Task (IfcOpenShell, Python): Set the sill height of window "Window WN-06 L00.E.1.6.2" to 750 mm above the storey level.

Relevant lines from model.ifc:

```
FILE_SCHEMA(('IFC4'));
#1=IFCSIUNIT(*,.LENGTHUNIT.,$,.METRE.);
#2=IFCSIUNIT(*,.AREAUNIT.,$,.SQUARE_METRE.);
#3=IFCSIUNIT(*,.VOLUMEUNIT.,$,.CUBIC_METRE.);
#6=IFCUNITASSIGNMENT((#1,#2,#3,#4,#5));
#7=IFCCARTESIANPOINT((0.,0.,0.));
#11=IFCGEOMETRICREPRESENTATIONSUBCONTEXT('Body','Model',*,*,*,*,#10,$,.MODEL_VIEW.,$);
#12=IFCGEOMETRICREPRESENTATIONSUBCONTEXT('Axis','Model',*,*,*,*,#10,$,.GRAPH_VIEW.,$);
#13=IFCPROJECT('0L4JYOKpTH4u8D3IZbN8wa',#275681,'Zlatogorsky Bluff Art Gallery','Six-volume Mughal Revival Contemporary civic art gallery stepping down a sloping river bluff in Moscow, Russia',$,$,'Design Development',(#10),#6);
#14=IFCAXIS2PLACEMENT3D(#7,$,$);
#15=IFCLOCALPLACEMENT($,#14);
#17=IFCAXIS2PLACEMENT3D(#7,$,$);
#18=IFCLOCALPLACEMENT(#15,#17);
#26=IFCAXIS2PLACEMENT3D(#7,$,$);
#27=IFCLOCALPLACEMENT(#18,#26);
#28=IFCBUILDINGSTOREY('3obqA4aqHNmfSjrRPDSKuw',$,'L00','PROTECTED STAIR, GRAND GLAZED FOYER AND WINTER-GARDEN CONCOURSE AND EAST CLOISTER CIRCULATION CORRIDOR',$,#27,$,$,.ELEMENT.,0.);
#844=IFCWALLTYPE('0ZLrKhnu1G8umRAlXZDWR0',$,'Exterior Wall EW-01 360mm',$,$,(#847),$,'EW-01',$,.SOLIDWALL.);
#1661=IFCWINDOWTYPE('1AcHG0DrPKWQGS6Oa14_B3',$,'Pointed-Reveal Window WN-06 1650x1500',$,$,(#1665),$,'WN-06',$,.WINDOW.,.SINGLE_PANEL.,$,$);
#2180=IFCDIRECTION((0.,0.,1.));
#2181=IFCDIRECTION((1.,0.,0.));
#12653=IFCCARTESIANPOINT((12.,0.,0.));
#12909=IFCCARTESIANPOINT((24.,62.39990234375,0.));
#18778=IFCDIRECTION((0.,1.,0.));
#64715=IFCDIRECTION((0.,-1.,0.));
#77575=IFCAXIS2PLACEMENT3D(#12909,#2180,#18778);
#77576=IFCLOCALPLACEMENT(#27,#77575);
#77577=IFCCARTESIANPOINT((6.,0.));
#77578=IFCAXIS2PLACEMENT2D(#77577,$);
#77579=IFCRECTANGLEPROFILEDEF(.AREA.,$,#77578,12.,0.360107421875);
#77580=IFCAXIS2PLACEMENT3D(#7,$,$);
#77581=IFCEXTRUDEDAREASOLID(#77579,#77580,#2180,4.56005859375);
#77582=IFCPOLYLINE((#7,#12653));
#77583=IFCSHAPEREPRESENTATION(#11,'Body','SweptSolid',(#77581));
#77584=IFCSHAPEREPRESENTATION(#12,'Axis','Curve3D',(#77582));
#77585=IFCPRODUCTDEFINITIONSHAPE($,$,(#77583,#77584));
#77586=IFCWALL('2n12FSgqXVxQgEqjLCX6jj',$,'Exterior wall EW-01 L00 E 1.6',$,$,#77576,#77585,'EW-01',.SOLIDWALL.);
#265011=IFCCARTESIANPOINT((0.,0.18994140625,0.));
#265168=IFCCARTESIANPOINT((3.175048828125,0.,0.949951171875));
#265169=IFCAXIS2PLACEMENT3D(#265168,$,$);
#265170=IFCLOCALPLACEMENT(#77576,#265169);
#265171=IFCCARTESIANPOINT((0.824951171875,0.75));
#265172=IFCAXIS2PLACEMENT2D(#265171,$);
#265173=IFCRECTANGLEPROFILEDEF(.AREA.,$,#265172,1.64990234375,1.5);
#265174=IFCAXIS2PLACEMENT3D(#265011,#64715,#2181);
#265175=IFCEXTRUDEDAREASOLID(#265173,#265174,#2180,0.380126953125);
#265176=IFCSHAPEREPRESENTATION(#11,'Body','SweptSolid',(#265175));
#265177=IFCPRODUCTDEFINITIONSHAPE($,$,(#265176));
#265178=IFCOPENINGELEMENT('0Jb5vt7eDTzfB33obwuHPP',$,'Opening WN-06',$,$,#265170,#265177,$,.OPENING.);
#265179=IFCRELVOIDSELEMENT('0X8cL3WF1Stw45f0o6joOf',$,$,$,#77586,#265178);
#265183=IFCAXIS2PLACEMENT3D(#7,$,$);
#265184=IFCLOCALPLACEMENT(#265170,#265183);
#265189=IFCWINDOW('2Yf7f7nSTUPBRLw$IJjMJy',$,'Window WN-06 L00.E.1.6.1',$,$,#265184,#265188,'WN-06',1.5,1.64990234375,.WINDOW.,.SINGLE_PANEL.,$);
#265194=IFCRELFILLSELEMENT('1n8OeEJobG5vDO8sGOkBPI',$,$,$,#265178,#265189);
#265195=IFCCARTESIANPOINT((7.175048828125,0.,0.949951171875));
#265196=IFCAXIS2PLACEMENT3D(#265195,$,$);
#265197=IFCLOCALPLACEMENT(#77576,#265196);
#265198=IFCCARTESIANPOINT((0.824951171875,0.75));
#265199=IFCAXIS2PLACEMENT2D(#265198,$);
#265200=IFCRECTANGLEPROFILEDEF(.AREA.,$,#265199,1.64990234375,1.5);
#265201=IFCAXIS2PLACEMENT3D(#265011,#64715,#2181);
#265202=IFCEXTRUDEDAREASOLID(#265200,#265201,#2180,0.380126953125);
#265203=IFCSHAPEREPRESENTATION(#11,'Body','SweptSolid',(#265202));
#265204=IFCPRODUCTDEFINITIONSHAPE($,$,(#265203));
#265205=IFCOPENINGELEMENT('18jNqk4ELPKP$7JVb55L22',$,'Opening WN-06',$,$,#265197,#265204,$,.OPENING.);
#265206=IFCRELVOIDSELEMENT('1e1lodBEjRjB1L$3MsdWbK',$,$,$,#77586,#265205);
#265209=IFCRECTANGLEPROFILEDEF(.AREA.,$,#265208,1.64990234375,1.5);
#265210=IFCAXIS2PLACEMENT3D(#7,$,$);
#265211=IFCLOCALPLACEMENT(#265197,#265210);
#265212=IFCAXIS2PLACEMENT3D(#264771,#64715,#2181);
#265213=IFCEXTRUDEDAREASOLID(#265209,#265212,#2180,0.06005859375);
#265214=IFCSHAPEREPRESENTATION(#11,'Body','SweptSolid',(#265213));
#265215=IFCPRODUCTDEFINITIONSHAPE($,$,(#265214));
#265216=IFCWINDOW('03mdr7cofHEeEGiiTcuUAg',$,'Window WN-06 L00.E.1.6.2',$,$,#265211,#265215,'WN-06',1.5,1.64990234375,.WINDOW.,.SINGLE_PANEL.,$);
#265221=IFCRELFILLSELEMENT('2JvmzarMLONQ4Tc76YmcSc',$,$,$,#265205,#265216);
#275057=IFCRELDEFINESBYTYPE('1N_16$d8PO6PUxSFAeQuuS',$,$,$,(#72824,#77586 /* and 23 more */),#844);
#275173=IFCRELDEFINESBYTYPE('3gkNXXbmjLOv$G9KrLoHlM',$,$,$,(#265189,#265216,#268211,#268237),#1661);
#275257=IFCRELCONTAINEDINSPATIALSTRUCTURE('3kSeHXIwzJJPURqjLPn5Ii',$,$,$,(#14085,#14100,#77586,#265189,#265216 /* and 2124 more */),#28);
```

```python
import numpy as np
import ifcopenshell
import ifcopenshell.api.geometry
import ifcopenshell.geom
import ifcopenshell.util.element
import ifcopenshell.util.placement
import ifcopenshell.util.shape
import ifcopenshell.util.unit

model = ifcopenshell.open("model.ifc")
unit_scale = ifcopenshell.util.unit.calculate_unit_scale(model)

window = model.by_guid("03mdr7cofHEeEGiiTcuUAg")
opening = window.FillsVoids[0].RelatingOpeningElement
storey = ifcopenshell.util.element.get_container(window, ifc_class="IfcBuildingStorey")
level = ifcopenshell.util.placement.get_local_placement(storey.ObjectPlacement)[2, 3]

# The opening's origin need not be at the sill, so measure its lowest point.
shape = ifcopenshell.geom.create_shape(ifcopenshell.geom.settings(), opening)
bottom = ifcopenshell.util.shape.get_shape_bottom_elevation(shape, shape.geometry) / unit_scale
dz = level + 0.75 - bottom

shift = np.array([0.0, 0.0, dz])
# The window is placed relative to its opening, so it follows when the opening moves.
matrix = ifcopenshell.util.placement.get_local_placement(opening.ObjectPlacement)
matrix[:3, 3] += shift
ifcopenshell.api.geometry.edit_object_placement(
    model, product=opening, matrix=matrix, is_si=False, should_transform_children=True
)

print(f"moved by {dz * unit_scale:+.3f} m")

model.write("model-out.ifc")
```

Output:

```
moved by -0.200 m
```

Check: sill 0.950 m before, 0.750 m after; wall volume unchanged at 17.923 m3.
